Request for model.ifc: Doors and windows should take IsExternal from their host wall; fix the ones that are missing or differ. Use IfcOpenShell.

First a look at what the model holds.

```python
import ifcopenshell
import ifcopenshell.util.element

model = ifcopenshell.open("model.ifc")
print(model.schema)
seen = {}
for e in model.by_type("IfcDoor") + model.by_type("IfcWindow"):
    if not e.FillsVoids:
        continue
    host = e.FillsVoids[0].RelatingOpeningElement.VoidsElements[0].RelatingBuildingElement
    own = ifcopenshell.util.element.get_pset(e, f"Pset_{e.is_a()[3:].removesuffix('StandardCase')}Common", "IsExternal")
    wall = ifcopenshell.util.element.get_pset(host, "Pset_WallCommon", "IsExternal")
    seen[e.is_a(), own, wall] = seen.get((e.is_a(), own, wall), 0) + 1
for (cls, own, wall), count in sorted(seen.items(), key=str):
    print(count, cls, "IsExternal:", own, "| host wall:", wall)
```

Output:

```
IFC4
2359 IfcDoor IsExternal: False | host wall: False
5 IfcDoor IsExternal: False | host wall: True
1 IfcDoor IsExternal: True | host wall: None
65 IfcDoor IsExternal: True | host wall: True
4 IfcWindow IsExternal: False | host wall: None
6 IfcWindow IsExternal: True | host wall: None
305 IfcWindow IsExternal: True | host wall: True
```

```python
import ifcopenshell
import ifcopenshell.api.pset
import ifcopenshell.util.element

model = ifcopenshell.open("model.ifc")

count = 0
for ifc_class, pset_name in (("IfcDoor", "Pset_DoorCommon"), ("IfcWindow", "Pset_WindowCommon")):
    for e in model.by_type(ifc_class):
        if not e.FillsVoids:
            continue
        host = e.FillsVoids[0].RelatingOpeningElement.VoidsElements[0].RelatingBuildingElement
        external = ifcopenshell.util.element.get_pset(host, "Pset_WallCommon", "IsExternal")
        if external is None or ifcopenshell.util.element.get_pset(e, pset_name, "IsExternal") == external:
            continue
        found = ifcopenshell.util.element.get_pset(e, pset_name, should_inherit=False)
        if found:
            pset = model.by_id(found["id"])
            if len(ifcopenshell.util.element.get_elements_by_pset(pset)) > 1:
                pset = ifcopenshell.api.pset.unshare_pset(model, products=[e], pset=pset)[0]
        else:
            pset = ifcopenshell.api.pset.add_pset(model, product=e, name=pset_name)
        ifcopenshell.api.pset.edit_pset(model, pset=pset, properties={"IsExternal": external})
        count += 1

print(count, "updated")

model.write("model_rev.ifc")
```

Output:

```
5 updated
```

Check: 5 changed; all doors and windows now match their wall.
